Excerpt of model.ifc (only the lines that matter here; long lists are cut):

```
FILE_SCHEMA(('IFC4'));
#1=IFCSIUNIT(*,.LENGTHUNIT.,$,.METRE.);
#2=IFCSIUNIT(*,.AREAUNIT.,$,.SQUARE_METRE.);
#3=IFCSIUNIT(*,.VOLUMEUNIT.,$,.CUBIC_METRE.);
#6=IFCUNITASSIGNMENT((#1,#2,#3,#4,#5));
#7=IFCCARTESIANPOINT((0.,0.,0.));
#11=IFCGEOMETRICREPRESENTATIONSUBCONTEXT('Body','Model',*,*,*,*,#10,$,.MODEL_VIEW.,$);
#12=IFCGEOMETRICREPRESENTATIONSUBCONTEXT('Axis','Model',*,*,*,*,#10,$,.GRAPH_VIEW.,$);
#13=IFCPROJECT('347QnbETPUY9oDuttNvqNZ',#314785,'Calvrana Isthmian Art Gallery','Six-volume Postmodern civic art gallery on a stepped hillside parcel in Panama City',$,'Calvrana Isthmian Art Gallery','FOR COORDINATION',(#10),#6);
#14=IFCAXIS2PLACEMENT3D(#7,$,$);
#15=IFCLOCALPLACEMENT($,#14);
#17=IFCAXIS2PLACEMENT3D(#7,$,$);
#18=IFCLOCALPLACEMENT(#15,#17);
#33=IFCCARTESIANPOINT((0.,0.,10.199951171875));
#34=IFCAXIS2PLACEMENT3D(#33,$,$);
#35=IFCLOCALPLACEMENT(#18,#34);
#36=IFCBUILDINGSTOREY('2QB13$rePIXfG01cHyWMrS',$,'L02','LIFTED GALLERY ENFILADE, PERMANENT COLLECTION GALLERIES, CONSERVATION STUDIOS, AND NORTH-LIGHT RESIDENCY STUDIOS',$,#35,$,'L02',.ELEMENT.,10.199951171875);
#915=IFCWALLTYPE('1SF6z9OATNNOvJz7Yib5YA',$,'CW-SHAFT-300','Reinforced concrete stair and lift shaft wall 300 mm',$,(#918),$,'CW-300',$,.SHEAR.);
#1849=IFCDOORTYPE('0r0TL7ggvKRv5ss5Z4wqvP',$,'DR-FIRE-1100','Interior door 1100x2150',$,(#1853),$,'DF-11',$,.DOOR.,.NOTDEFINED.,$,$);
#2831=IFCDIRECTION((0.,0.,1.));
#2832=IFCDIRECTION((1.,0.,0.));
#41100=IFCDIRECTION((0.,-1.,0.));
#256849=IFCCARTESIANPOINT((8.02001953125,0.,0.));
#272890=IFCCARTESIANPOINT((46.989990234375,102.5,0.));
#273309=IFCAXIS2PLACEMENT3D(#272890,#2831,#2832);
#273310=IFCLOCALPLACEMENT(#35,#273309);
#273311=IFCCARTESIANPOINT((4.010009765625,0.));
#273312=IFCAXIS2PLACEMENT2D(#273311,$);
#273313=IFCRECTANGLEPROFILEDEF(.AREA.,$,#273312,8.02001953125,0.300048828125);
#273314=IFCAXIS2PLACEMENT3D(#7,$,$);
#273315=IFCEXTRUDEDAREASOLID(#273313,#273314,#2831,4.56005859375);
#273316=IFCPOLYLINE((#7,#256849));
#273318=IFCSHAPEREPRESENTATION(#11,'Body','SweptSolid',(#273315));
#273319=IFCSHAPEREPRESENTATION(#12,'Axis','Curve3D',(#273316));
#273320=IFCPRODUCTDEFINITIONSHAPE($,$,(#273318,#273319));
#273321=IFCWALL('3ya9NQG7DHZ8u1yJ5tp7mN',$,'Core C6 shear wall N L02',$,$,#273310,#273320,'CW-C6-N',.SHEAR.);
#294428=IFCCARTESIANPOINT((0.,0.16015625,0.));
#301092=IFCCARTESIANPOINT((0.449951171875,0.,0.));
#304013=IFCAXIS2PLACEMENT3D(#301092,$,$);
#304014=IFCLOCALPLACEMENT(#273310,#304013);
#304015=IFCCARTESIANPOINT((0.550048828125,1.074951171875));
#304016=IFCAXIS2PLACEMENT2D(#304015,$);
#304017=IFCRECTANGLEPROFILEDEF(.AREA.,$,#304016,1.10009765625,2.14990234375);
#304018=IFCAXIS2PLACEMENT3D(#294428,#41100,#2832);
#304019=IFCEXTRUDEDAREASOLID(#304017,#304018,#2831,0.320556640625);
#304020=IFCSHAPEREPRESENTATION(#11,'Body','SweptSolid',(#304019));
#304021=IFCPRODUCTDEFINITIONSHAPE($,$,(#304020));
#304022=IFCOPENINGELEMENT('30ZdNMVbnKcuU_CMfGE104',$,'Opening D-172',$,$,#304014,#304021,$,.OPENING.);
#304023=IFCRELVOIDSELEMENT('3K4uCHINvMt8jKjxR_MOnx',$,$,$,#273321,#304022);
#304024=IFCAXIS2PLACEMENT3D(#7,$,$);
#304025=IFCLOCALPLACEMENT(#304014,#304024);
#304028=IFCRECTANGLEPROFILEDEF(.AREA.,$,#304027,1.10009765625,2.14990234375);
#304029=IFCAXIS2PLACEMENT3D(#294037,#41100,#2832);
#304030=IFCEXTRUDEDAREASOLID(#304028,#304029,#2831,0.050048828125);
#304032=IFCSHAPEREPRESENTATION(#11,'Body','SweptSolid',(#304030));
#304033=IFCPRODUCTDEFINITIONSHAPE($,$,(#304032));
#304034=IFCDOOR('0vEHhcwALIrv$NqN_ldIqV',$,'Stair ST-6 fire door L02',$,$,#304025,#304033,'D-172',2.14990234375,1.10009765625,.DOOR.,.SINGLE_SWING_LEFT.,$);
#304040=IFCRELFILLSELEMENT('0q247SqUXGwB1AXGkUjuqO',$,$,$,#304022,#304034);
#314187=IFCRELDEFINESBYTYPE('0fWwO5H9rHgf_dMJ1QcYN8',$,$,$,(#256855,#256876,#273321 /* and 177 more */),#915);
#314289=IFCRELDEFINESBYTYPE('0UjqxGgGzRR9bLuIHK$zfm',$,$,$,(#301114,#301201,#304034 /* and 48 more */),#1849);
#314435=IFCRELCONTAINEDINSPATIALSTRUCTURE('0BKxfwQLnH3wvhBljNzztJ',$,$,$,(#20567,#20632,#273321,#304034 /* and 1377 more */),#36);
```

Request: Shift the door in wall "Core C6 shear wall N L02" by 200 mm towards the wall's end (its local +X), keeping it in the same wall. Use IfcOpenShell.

```python
import ifcopenshell
import ifcopenshell.api.geometry
import ifcopenshell.util.placement
import ifcopenshell.util.unit

model = ifcopenshell.open("model.ifc")
unit_scale = ifcopenshell.util.unit.calculate_unit_scale(model)

door = model.by_guid("0vEHhcwALIrv$NqN_ldIqV")
opening = door.FillsVoids[0].RelatingOpeningElement
wall = opening.VoidsElements[0].RelatingBuildingElement

wall_matrix = ifcopenshell.util.placement.get_local_placement(wall.ObjectPlacement)
shift = wall_matrix[:3, 0] * 0.2 / unit_scale
before = ifcopenshell.util.placement.get_local_placement(door.ObjectPlacement)[:3, 3].copy()

# The door is placed relative to its opening, so it follows when the opening moves.
matrix = ifcopenshell.util.placement.get_local_placement(opening.ObjectPlacement)
matrix[:3, 3] += shift
ifcopenshell.api.geometry.edit_object_placement(
    model, product=opening, matrix=matrix, is_si=False, should_transform_children=True
)

after = ifcopenshell.util.placement.get_local_placement(door.ObjectPlacement)[:3, 3]
print("door moved by", (after - before).round(3) + 0.0)

model.write("model-out.ifc")
```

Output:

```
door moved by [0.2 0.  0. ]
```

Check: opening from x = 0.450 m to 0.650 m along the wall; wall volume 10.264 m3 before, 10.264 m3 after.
